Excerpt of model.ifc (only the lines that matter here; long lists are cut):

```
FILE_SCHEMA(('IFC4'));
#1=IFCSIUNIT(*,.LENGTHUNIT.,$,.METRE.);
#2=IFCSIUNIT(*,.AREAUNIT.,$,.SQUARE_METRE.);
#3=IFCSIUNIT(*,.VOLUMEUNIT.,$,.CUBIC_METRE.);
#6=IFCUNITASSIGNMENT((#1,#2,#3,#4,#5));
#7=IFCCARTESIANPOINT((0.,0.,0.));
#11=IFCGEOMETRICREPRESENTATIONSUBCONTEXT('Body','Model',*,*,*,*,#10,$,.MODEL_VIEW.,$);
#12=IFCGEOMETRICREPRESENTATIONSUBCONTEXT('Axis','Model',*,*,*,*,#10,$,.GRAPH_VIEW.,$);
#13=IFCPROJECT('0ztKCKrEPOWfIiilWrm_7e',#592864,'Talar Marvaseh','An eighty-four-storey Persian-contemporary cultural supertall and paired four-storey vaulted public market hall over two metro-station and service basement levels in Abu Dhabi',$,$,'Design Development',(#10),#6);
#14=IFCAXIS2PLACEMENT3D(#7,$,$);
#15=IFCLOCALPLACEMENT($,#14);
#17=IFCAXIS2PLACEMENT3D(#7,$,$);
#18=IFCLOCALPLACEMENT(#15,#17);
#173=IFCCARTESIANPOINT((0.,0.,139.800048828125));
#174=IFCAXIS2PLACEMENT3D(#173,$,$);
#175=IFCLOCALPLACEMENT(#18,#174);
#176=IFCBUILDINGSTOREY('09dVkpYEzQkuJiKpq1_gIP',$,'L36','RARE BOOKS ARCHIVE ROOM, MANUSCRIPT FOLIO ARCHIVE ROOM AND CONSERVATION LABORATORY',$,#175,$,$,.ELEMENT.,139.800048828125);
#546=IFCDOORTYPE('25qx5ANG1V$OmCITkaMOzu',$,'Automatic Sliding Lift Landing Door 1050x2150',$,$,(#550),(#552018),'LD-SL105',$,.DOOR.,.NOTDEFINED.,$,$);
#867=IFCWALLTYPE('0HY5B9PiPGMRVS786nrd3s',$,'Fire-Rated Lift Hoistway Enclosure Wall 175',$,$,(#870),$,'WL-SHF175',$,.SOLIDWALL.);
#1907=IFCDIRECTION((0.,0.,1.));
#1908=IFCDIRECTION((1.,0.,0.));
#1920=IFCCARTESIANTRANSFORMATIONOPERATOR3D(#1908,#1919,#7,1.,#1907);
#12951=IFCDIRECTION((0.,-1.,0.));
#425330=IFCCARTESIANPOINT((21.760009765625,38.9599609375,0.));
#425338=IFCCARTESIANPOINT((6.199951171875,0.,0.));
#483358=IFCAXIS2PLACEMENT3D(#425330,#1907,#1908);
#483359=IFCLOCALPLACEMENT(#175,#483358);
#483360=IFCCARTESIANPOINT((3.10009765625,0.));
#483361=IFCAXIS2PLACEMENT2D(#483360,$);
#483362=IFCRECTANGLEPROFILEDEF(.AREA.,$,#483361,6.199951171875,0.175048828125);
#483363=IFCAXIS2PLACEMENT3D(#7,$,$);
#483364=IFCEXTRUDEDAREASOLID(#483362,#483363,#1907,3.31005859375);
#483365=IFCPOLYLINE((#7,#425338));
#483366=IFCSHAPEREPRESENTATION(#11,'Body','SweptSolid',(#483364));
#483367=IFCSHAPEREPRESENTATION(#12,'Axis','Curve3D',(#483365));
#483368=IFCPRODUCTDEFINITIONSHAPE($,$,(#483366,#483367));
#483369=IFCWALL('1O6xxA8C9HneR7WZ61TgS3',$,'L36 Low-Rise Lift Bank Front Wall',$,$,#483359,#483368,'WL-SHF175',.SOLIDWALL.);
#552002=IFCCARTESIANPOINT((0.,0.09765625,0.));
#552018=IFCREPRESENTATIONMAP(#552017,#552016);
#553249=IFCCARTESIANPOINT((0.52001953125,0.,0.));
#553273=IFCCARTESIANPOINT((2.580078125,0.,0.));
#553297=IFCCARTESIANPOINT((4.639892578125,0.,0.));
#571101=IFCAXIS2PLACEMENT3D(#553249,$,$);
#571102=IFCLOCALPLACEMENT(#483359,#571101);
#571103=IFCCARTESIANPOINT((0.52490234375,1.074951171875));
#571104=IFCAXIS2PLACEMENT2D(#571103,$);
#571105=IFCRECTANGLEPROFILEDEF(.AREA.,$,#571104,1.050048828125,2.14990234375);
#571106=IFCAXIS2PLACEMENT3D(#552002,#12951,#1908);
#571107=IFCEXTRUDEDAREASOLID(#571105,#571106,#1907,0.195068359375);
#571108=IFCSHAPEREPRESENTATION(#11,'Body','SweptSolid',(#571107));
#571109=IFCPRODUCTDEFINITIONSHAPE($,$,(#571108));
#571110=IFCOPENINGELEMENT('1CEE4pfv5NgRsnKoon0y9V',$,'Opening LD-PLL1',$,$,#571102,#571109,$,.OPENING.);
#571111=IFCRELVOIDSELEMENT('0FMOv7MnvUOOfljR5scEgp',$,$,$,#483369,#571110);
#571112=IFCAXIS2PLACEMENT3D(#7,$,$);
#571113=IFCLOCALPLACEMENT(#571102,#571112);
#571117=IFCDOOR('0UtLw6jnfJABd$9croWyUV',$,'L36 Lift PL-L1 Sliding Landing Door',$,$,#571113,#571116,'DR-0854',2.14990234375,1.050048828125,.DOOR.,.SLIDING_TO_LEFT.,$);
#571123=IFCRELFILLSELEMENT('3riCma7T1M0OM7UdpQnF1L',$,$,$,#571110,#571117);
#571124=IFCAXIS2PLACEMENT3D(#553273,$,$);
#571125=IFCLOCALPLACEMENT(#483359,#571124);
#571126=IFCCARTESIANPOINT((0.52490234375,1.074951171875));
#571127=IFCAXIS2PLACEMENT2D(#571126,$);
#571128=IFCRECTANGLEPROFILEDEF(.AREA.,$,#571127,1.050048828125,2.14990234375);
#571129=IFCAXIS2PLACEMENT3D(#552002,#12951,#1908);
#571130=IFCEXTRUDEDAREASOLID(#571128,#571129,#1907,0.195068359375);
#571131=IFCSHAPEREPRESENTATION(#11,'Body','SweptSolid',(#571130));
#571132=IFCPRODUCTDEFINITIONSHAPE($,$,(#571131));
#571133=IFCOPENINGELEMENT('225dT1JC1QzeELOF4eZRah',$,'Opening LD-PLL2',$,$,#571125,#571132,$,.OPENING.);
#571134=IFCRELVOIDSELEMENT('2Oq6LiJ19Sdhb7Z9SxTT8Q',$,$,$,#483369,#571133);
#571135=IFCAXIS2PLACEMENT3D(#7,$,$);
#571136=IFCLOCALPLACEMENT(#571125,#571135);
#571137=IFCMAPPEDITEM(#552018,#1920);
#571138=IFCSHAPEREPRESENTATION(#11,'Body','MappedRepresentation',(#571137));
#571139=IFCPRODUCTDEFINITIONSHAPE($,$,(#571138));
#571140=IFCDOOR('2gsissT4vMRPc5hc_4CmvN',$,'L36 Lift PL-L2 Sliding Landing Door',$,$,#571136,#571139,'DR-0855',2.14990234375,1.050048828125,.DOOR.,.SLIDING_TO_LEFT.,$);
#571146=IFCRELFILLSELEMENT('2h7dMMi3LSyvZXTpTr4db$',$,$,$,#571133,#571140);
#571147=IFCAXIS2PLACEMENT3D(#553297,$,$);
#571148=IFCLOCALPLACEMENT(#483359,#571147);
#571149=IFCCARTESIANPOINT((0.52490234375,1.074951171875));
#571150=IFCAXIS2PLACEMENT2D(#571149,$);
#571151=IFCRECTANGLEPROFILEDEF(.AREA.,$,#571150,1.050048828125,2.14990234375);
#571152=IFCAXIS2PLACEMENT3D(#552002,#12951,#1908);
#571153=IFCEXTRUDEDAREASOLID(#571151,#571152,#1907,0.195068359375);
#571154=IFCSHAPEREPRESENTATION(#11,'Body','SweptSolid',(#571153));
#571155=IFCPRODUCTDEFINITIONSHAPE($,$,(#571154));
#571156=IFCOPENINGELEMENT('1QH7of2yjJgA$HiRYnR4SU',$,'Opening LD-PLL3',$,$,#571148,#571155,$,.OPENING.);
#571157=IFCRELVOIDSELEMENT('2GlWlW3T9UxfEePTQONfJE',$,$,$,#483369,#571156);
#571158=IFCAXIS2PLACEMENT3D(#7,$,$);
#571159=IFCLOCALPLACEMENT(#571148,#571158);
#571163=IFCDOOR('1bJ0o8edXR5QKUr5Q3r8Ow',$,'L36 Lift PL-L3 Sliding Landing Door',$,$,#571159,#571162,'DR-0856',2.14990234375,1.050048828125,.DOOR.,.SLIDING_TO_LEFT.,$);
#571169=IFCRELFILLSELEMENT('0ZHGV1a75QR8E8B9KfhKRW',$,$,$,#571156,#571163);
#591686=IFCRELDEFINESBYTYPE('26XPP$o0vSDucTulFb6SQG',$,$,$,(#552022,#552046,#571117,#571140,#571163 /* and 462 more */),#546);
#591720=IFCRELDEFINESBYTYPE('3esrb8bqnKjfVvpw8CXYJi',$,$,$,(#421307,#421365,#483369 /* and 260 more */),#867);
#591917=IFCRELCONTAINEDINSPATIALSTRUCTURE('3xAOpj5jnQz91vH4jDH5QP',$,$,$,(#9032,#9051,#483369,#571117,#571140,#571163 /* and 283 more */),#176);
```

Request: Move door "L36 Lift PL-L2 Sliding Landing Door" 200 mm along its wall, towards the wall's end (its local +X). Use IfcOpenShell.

```python
import ifcopenshell
import ifcopenshell.api.geometry
import ifcopenshell.util.placement
import ifcopenshell.util.unit

model = ifcopenshell.open("model.ifc")
unit_scale = ifcopenshell.util.unit.calculate_unit_scale(model)

door = model.by_id(571140)
opening = door.FillsVoids[0].RelatingOpeningElement
wall = opening.VoidsElements[0].RelatingBuildingElement

wall_matrix = ifcopenshell.util.placement.get_local_placement(wall.ObjectPlacement)
shift = wall_matrix[:3, 0] * 0.2 / unit_scale
before = ifcopenshell.util.placement.get_local_placement(door.ObjectPlacement)[:3, 3].copy()

# The door is placed relative to its opening, so it follows when the opening moves.
matrix = ifcopenshell.util.placement.get_local_placement(opening.ObjectPlacement)
matrix[:3, 3] += shift
ifcopenshell.api.geometry.edit_object_placement(
    model, product=opening, matrix=matrix, is_si=False, should_transform_children=True
)

after = ifcopenshell.util.placement.get_local_placement(door.ObjectPlacement)[:3, 3]
print("door moved by", (after - before).round(3) + 0.0)

model.write("model_rev.ifc")
```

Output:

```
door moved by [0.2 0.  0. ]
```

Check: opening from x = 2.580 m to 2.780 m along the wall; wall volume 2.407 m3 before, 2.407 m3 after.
